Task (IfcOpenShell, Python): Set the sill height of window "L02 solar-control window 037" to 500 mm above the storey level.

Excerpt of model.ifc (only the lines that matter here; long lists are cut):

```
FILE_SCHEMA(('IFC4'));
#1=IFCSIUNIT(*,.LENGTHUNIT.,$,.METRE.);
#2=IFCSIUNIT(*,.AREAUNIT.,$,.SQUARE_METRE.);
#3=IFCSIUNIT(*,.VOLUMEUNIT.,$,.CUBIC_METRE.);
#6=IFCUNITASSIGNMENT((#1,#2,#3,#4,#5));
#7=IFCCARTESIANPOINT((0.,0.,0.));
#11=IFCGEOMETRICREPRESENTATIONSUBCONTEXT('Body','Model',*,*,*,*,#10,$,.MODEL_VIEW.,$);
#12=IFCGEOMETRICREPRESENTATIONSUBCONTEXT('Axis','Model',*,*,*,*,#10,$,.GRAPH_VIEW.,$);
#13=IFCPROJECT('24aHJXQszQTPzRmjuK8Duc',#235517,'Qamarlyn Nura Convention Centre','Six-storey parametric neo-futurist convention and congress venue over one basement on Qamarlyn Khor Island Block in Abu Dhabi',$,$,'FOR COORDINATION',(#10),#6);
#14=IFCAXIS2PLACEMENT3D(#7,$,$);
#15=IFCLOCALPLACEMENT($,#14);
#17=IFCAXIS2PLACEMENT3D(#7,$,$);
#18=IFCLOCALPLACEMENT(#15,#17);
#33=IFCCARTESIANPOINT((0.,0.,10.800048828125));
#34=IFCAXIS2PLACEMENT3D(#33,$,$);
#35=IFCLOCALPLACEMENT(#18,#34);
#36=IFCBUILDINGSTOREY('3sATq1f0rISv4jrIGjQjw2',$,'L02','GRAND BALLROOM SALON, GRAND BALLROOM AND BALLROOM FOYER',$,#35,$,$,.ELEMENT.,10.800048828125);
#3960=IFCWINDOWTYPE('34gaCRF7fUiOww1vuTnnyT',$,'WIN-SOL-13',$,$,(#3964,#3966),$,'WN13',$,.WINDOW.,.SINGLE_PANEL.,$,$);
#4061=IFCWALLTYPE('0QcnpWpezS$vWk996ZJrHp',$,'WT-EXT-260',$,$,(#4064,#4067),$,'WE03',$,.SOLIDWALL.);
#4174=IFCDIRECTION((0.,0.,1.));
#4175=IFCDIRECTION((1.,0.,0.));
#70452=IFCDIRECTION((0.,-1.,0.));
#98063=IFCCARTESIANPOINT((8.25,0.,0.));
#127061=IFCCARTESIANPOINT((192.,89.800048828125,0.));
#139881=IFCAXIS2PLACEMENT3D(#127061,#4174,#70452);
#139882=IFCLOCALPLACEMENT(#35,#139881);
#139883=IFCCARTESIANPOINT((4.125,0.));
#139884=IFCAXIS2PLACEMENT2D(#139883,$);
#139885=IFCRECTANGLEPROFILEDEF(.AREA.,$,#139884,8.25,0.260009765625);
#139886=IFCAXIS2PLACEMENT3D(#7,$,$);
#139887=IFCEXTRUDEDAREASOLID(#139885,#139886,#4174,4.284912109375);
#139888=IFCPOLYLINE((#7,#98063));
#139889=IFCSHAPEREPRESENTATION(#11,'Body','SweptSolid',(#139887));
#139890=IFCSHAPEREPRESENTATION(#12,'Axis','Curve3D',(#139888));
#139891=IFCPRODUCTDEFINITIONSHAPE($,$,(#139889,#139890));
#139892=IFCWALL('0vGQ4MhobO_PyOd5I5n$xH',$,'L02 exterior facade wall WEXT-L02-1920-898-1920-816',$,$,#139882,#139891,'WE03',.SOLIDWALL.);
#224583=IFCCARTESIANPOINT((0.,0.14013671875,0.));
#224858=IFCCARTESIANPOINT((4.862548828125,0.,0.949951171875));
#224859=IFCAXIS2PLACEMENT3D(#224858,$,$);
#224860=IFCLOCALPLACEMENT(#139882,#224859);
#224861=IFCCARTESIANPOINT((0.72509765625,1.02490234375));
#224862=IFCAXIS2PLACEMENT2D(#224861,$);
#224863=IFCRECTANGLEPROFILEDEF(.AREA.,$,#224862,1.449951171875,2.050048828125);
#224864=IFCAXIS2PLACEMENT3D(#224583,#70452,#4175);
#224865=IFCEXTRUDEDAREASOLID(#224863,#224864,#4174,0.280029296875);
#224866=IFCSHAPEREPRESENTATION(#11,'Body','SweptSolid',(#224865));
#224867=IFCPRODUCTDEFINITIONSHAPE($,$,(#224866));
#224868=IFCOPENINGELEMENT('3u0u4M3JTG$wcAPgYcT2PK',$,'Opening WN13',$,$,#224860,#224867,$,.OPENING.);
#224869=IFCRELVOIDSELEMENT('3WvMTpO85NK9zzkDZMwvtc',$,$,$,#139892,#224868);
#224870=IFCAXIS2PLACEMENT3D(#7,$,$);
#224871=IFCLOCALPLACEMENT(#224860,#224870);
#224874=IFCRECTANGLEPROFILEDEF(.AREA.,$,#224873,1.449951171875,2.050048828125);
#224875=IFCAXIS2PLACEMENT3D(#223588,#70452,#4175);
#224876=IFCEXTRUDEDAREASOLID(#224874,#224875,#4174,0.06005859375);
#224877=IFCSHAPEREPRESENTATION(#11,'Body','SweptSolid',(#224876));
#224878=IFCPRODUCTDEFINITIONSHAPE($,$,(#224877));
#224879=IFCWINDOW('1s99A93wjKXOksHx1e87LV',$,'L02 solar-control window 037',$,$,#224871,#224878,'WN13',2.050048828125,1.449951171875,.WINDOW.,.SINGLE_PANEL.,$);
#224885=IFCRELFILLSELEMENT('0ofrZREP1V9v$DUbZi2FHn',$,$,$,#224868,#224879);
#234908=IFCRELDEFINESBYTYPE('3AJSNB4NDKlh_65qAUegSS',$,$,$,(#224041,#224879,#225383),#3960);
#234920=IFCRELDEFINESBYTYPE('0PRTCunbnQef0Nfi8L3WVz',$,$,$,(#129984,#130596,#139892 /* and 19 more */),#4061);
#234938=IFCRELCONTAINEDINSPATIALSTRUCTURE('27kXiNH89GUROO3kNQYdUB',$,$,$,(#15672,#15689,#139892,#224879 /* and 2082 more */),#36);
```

```python
import numpy as np
import ifcopenshell
import ifcopenshell.api.geometry
import ifcopenshell.geom
import ifcopenshell.util.element
import ifcopenshell.util.placement
import ifcopenshell.util.shape
import ifcopenshell.util.unit

model = ifcopenshell.open("model.ifc")
unit_scale = ifcopenshell.util.unit.calculate_unit_scale(model)

window = model.by_guid("1s99A93wjKXOksHx1e87LV")
opening = window.FillsVoids[0].RelatingOpeningElement
storey = ifcopenshell.util.element.get_container(window, ifc_class="IfcBuildingStorey")
level = ifcopenshell.util.placement.get_local_placement(storey.ObjectPlacement)[2, 3]

# The opening's origin need not be at the sill, so measure its lowest point.
shape = ifcopenshell.geom.create_shape(ifcopenshell.geom.settings(), opening)
bottom = ifcopenshell.util.shape.get_shape_bottom_elevation(shape, shape.geometry) / unit_scale
dz = level + 0.5 / unit_scale - bottom

shift = np.array([0.0, 0.0, dz])
# The window is placed relative to its opening, so it follows when the opening moves.
matrix = ifcopenshell.util.placement.get_local_placement(opening.ObjectPlacement)
matrix[:3, 3] += shift
ifcopenshell.api.geometry.edit_object_placement(
    model, product=opening, matrix=matrix, is_si=False, should_transform_children=True
)

print(f"moved by {dz * unit_scale:+.3f} m")

model.write("model_v2.ifc")
```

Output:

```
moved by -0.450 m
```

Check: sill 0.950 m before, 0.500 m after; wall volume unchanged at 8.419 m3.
